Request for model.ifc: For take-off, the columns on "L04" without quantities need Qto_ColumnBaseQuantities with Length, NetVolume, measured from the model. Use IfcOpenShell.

First a look at what the model holds.

```python
import ifcopenshell
import ifcopenshell.util.element
import ifcopenshell.util.unit

model = ifcopenshell.open("model.ifc")
print(model.schema)
for unit_type in ("LENGTHUNIT", "AREAUNIT", "VOLUMEUNIT"):
    print(unit_type, ifcopenshell.util.unit.calculate_unit_scale(model, unit_type))
storey = next(s for s in model.by_type("IfcBuildingStorey") if s.Name == "L04")
columns = [e for e in ifcopenshell.util.element.get_decomposition(storey) if e.is_a("IfcColumn")]
for e in sorted(columns, key=lambda e: e.id()):
    print(e.id(), e.is_a(), e.Name, list(ifcopenshell.util.element.get_psets(e, qtos_only=True)), sep=" | ")
```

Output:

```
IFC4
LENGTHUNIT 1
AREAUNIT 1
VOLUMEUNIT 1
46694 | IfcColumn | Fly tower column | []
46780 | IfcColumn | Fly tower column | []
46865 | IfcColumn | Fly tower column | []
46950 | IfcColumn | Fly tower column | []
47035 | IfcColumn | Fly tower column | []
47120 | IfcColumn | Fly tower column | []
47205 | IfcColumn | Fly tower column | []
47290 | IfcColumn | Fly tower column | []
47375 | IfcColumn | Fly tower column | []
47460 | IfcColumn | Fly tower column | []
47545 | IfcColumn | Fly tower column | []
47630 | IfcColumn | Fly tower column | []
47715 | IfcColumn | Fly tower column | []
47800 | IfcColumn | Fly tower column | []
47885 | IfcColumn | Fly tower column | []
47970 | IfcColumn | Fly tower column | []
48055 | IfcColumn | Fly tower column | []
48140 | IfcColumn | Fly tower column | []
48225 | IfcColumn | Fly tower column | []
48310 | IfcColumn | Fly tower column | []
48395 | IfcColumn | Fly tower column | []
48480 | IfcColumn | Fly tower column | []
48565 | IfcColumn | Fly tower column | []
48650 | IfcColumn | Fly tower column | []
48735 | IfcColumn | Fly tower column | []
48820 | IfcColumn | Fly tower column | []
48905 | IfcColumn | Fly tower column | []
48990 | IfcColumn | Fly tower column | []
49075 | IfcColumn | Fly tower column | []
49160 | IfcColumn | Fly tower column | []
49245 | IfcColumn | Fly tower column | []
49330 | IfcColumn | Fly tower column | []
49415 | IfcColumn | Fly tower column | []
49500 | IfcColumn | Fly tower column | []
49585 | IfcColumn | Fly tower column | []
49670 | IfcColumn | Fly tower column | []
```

```python
import ifcopenshell
import ifcopenshell.api.pset
import ifcopenshell.geom
import ifcopenshell.util.element
import ifcopenshell.util.shape
import ifcopenshell.util.unit

model = ifcopenshell.open("model.ifc")
unit_scale = ifcopenshell.util.unit.calculate_unit_scale(model)
volume_scale = ifcopenshell.util.unit.calculate_unit_scale(model, "VOLUMEUNIT")
settings = ifcopenshell.geom.settings()

storey = next(s for s in model.by_type("IfcBuildingStorey") if s.Name == "L04")
columns = [e for e in ifcopenshell.util.element.get_decomposition(storey) if e.is_a("IfcColumn")]

for e in sorted(columns, key=lambda e: e.id()):
    if ifcopenshell.util.element.get_psets(e, qtos_only=True, should_inherit=False):
        continue
    # Geometry comes back in metres, in the element's own axes.
    shape = ifcopenshell.geom.create_shape(settings, e)
    values = {
        "Length": ifcopenshell.util.shape.get_z(shape.geometry) / unit_scale,
        "NetVolume": ifcopenshell.util.shape.get_volume(shape.geometry) / volume_scale,
    }
    qto = ifcopenshell.api.pset.add_qto(model, product=e, name="Qto_ColumnBaseQuantities")
    ifcopenshell.api.pset.edit_qto(model, qto=qto, properties=values)
    print(e.id(), {k: round(v, 3) for k, v in values.items()})

model.write("model_updated.ifc")
```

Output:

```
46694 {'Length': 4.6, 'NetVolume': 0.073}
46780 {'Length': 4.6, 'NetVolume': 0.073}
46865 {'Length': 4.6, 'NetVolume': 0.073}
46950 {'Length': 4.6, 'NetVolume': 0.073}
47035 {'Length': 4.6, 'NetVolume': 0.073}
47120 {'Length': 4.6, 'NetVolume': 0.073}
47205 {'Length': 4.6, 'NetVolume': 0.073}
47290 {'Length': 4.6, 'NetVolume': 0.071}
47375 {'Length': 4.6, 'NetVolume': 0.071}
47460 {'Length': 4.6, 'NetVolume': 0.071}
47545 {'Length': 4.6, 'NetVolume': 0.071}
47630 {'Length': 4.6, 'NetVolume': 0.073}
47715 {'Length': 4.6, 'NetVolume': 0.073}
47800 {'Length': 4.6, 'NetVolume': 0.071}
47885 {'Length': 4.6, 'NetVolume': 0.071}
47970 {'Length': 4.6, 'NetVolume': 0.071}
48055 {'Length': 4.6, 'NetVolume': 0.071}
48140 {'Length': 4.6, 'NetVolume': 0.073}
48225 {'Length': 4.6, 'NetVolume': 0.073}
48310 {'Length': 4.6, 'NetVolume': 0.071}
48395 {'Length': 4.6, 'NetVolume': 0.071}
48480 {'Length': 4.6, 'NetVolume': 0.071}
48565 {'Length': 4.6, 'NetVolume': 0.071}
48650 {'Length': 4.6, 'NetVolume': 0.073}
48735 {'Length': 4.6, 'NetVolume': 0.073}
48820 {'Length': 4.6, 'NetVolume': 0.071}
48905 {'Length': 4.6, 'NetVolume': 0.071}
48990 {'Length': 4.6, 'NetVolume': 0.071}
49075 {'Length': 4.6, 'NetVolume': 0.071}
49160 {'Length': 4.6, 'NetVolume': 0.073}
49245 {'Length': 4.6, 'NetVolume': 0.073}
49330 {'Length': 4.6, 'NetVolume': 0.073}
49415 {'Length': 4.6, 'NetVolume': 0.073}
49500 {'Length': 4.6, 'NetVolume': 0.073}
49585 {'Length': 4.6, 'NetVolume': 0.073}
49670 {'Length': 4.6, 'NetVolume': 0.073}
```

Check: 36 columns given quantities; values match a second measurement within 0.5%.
